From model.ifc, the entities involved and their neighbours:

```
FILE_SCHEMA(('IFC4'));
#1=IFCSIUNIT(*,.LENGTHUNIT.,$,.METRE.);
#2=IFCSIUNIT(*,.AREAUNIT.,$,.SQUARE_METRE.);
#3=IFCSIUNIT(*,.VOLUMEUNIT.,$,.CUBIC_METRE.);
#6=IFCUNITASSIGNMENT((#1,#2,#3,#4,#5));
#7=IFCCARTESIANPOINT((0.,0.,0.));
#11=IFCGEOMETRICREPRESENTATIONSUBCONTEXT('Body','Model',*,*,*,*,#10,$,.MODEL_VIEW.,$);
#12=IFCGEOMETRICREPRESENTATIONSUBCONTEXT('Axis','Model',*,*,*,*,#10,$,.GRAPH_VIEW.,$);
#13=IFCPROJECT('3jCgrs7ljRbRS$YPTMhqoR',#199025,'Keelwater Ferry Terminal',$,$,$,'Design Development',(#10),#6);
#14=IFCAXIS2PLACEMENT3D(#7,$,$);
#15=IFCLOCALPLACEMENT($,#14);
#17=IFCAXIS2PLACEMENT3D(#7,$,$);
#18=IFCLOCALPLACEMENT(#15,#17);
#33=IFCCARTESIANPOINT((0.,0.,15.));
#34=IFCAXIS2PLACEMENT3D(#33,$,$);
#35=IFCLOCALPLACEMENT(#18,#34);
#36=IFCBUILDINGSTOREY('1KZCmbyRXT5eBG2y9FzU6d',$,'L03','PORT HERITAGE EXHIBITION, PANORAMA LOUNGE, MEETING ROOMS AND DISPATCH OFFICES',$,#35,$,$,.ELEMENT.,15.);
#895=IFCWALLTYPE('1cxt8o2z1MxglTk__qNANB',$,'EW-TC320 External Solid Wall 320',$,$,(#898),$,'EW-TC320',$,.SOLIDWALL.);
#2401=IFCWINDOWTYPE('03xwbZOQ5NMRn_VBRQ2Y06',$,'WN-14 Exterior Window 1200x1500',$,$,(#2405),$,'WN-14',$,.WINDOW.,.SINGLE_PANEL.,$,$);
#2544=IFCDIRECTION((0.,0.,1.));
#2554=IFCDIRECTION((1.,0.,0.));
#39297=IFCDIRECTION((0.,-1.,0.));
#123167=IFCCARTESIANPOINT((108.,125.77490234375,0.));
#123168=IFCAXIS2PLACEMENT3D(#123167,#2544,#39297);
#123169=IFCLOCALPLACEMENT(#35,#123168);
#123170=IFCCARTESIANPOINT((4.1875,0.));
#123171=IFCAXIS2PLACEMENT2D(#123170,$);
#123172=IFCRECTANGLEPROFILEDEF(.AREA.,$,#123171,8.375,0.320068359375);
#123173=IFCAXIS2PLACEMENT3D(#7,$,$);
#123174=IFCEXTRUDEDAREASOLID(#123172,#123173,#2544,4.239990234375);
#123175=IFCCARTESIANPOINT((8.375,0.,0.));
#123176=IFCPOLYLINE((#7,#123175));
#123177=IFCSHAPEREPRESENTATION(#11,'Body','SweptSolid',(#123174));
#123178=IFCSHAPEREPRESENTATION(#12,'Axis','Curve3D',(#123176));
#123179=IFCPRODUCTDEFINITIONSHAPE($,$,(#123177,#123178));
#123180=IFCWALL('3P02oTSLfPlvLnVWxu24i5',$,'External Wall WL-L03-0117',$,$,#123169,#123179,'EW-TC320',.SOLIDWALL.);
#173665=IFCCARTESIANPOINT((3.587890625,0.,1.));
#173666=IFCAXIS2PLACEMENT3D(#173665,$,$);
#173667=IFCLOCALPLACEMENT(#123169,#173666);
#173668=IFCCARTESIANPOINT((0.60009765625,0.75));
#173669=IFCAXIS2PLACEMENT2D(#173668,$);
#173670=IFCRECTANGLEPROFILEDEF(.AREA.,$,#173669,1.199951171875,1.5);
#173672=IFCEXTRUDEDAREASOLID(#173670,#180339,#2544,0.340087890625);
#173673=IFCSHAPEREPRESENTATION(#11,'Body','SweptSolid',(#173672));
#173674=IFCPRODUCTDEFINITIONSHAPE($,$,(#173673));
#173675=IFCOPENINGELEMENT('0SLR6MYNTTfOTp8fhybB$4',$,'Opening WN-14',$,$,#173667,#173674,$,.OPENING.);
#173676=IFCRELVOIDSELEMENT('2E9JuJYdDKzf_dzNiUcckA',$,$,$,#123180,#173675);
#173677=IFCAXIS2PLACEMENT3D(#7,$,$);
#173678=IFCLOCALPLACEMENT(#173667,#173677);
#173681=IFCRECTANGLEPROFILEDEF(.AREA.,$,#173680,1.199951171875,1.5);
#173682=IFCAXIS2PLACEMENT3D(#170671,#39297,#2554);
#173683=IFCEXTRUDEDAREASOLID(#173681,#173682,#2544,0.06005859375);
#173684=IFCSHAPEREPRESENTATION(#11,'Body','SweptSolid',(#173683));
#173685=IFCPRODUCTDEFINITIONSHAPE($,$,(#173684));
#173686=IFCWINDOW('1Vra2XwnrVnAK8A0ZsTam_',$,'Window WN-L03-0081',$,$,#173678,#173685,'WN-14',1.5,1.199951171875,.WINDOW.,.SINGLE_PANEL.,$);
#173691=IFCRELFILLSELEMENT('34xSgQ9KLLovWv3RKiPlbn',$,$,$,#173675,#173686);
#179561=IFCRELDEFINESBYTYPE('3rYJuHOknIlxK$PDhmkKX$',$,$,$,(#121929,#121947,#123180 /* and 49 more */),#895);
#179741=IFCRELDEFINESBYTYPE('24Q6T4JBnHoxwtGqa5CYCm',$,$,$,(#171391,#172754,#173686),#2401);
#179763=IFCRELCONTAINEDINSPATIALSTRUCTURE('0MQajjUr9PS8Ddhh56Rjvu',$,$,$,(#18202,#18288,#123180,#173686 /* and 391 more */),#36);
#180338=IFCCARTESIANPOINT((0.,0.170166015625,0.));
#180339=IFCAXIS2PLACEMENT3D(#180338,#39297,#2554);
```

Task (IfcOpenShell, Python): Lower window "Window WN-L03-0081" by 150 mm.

```python
import numpy as np
import ifcopenshell
import ifcopenshell.api.geometry
import ifcopenshell.util.placement
import ifcopenshell.util.unit

model = ifcopenshell.open("model.ifc")
unit_scale = ifcopenshell.util.unit.calculate_unit_scale(model)

window = model.by_guid("1Vra2XwnrVnAK8A0ZsTam_")
opening = window.FillsVoids[0].RelatingOpeningElement
dz = -0.15 / unit_scale

shift = np.array([0.0, 0.0, dz])
# The window is placed relative to its opening, so it follows when the opening moves.
matrix = ifcopenshell.util.placement.get_local_placement(opening.ObjectPlacement)
matrix[:3, 3] += shift
ifcopenshell.api.geometry.edit_object_placement(
    model, product=opening, matrix=matrix, is_si=False, should_transform_children=True
)

print(f"moved by {dz * unit_scale:+.3f} m")

model.write("model_rev.ifc")
```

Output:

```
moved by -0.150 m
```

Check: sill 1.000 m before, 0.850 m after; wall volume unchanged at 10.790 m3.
